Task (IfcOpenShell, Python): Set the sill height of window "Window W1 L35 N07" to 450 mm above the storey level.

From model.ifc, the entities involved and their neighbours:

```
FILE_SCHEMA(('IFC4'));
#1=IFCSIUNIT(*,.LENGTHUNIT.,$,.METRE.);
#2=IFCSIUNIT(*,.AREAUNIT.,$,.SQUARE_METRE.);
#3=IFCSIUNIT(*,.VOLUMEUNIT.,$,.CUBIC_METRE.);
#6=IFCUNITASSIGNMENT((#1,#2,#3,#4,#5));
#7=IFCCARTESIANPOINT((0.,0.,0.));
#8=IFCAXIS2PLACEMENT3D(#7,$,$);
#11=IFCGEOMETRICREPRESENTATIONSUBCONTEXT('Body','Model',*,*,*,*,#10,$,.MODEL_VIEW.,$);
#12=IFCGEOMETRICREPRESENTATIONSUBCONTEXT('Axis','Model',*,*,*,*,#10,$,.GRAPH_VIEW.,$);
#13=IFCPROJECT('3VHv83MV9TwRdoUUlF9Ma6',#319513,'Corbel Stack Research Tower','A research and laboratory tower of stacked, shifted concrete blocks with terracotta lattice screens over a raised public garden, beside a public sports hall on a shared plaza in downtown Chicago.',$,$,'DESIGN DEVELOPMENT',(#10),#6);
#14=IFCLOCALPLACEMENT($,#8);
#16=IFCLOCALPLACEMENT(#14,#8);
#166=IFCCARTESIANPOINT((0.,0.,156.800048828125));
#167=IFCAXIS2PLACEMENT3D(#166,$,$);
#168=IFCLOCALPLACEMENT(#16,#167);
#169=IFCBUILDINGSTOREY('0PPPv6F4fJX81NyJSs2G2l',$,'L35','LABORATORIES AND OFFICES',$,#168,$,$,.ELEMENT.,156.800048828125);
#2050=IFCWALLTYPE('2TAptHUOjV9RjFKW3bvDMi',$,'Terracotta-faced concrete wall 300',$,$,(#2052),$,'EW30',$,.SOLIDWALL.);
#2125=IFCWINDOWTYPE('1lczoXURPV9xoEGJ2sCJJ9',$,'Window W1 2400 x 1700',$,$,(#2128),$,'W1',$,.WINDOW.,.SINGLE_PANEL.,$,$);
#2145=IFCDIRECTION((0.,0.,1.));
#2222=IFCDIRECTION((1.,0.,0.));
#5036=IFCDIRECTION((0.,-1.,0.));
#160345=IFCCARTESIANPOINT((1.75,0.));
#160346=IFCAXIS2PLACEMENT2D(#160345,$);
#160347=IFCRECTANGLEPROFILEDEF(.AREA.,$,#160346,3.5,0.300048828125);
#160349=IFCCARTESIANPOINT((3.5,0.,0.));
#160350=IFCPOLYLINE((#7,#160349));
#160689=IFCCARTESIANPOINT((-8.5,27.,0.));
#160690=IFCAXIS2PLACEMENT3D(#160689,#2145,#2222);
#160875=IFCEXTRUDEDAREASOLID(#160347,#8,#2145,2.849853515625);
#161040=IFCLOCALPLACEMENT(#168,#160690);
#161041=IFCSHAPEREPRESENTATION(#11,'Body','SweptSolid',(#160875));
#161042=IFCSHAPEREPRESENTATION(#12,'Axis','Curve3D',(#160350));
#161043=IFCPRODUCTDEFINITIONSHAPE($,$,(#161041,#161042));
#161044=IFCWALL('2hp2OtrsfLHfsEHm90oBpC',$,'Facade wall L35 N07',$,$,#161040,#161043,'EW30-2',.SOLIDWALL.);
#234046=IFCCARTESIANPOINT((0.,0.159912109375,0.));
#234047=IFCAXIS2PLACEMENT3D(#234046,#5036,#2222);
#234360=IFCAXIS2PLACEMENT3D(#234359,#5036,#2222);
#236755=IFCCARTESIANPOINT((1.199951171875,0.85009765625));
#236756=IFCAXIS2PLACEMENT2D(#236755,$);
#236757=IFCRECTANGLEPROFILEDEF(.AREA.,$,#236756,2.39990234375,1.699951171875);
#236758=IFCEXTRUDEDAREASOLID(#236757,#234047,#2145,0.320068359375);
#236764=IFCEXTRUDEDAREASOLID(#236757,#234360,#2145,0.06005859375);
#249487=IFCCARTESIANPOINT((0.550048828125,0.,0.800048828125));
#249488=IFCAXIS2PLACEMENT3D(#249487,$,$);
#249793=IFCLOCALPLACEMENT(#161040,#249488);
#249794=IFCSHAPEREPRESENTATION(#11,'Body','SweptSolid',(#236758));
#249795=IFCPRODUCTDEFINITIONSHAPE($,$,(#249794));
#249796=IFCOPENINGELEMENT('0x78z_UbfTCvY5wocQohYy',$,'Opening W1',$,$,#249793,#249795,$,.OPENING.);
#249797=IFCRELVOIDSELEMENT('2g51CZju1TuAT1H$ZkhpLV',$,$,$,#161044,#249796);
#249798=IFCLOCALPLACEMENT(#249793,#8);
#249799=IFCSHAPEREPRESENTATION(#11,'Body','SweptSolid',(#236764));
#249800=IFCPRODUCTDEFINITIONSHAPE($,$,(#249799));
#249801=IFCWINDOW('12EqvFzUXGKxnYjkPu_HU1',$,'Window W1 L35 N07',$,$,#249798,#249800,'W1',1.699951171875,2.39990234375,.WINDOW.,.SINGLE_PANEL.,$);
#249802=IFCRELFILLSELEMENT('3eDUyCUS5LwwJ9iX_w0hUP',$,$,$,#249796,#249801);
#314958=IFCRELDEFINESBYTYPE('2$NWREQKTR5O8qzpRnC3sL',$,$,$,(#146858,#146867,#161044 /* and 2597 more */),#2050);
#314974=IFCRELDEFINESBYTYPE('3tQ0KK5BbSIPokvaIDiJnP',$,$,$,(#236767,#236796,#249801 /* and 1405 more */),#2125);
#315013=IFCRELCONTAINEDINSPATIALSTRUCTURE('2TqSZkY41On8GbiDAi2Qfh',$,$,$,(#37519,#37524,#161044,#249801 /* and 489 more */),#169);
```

```python
import numpy as np
import ifcopenshell
import ifcopenshell.api.geometry
import ifcopenshell.geom
import ifcopenshell.util.element
import ifcopenshell.util.placement
import ifcopenshell.util.shape
import ifcopenshell.util.unit

model = ifcopenshell.open("model.ifc")
unit_scale = ifcopenshell.util.unit.calculate_unit_scale(model)

window = model.by_guid("12EqvFzUXGKxnYjkPu_HU1")
opening = window.FillsVoids[0].RelatingOpeningElement
storey = ifcopenshell.util.element.get_container(window, ifc_class="IfcBuildingStorey")
level = ifcopenshell.util.placement.get_local_placement(storey.ObjectPlacement)[2, 3]

# The opening's origin need not be at the sill, so measure its lowest point.
shape = ifcopenshell.geom.create_shape(ifcopenshell.geom.settings(), opening)
bottom = ifcopenshell.util.shape.get_shape_bottom_elevation(shape, shape.geometry) / unit_scale
dz = level + 0.45 / unit_scale - bottom

shift = np.array([0.0, 0.0, dz])
# The window is placed relative to its opening, so it follows when the opening moves.
matrix = ifcopenshell.util.placement.get_local_placement(opening.ObjectPlacement)
matrix[:3, 3] += shift
ifcopenshell.api.geometry.edit_object_placement(
    model, product=opening, matrix=matrix, is_si=False, should_transform_children=True
)

print(f"moved by {dz * unit_scale:+.3f} m")

model.write("model_rev.ifc")
```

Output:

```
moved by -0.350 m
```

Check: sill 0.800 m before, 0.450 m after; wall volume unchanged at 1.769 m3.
